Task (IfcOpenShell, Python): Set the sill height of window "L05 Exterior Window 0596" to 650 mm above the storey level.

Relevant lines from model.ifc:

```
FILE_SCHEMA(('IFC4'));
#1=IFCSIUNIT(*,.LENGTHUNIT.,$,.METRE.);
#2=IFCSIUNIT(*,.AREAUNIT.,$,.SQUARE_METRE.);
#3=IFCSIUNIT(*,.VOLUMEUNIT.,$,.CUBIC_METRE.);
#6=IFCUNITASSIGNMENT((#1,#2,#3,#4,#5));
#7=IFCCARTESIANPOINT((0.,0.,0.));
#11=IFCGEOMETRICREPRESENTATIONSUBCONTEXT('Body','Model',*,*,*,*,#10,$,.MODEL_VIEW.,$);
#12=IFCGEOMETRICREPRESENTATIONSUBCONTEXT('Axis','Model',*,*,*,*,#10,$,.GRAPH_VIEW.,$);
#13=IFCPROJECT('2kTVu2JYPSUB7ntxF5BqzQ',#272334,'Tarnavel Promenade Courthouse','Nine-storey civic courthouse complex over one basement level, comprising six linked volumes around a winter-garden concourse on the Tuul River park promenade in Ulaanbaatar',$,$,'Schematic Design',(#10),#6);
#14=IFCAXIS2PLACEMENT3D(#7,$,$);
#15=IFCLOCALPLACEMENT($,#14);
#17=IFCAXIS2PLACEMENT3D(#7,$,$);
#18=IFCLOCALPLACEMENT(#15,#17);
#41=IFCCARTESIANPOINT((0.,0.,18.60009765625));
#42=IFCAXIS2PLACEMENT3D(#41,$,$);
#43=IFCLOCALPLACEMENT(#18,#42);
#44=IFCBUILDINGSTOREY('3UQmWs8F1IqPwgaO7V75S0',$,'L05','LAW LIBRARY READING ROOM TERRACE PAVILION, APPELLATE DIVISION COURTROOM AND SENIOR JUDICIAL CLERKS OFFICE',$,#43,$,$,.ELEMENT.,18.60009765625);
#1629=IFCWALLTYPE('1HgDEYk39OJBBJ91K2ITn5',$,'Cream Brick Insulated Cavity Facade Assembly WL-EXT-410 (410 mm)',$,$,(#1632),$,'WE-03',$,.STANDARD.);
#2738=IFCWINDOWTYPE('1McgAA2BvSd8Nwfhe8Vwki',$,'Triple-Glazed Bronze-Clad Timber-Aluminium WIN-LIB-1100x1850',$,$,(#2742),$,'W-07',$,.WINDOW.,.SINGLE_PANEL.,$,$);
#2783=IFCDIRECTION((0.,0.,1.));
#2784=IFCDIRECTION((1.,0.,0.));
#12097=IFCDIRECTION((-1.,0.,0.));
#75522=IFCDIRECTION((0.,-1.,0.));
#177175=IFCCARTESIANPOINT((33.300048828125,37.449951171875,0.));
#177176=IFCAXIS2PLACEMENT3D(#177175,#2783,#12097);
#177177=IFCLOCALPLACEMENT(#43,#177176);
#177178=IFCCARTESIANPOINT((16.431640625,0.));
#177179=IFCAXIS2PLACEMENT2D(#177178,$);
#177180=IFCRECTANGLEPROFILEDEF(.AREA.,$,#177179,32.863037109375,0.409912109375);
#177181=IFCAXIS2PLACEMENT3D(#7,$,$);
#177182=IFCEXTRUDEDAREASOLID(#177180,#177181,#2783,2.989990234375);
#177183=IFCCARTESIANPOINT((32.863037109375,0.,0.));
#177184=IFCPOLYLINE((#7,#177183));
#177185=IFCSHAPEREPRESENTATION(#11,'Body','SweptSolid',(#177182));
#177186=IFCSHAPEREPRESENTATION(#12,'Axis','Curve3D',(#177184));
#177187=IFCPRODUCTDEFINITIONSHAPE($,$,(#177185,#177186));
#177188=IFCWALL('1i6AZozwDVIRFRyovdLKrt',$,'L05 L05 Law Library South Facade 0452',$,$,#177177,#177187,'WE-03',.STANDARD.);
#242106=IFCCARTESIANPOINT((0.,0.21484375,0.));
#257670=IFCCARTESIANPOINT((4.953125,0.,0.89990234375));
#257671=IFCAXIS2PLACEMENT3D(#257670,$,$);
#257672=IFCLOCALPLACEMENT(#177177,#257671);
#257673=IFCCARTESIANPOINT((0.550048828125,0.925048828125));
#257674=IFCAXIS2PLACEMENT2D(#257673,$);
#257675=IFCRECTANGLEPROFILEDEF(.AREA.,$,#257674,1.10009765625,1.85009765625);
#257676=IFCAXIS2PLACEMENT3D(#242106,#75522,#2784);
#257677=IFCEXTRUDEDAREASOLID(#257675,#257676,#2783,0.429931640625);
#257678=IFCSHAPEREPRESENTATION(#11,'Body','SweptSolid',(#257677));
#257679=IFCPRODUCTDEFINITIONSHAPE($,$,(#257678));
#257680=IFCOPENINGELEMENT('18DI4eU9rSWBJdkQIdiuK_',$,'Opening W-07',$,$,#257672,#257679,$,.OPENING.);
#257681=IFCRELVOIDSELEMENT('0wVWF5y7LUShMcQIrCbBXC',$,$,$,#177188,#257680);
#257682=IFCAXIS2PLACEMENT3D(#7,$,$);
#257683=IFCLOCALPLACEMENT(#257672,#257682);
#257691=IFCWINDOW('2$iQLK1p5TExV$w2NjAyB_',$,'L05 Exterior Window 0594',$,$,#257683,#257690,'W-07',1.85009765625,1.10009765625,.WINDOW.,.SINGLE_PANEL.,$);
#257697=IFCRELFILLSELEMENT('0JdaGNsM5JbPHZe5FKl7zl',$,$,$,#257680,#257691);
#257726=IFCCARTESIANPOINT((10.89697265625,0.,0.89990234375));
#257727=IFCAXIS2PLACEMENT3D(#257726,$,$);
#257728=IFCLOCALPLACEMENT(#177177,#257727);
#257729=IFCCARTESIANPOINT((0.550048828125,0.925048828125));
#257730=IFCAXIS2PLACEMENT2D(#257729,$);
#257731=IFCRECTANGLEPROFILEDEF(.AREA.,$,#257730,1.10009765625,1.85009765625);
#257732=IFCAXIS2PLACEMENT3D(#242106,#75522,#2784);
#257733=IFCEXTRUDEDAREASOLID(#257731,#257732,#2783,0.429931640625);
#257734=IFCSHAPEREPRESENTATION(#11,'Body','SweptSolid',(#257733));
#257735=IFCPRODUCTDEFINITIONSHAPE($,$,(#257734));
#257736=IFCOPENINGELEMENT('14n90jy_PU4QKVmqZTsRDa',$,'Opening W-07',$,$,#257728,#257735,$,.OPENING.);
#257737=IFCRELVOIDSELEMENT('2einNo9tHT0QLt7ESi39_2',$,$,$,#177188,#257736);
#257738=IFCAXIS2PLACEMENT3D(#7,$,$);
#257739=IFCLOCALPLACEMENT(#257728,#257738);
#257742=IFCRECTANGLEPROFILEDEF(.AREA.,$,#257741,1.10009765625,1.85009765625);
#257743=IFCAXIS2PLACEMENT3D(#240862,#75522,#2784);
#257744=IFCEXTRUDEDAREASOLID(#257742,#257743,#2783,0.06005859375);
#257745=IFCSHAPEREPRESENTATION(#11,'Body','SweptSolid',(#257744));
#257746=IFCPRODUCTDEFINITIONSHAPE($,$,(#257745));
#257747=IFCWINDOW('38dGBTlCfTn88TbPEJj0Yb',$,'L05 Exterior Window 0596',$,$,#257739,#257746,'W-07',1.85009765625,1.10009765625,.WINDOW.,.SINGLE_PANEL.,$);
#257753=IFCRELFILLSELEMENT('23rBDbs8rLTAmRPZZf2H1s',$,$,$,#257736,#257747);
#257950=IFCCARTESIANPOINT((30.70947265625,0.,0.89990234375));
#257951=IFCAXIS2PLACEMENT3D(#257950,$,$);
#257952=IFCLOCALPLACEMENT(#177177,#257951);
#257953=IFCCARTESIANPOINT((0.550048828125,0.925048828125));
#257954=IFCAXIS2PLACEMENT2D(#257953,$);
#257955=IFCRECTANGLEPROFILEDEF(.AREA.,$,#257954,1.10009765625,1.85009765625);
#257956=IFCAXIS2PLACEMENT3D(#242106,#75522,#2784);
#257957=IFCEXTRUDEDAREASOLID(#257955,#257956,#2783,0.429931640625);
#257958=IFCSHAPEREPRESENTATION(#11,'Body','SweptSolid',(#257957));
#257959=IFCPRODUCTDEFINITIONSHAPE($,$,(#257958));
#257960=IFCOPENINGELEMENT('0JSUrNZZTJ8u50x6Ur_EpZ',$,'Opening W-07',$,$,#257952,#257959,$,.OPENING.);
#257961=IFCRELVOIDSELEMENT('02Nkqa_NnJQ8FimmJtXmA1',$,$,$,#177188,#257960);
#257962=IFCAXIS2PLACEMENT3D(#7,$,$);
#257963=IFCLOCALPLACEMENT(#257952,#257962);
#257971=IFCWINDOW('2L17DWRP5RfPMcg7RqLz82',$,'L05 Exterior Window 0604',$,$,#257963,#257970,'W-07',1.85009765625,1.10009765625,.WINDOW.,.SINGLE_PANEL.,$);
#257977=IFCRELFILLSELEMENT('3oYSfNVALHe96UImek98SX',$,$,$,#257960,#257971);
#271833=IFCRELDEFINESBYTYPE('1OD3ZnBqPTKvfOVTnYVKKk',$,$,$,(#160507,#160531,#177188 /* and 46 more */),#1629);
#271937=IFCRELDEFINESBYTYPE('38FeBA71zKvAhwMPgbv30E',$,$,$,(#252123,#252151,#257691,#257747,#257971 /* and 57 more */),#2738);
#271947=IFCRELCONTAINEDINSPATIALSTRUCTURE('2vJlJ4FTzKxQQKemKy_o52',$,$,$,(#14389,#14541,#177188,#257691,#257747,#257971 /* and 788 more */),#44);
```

```python
import numpy as np
import ifcopenshell
import ifcopenshell.api.geometry
import ifcopenshell.geom
import ifcopenshell.util.element
import ifcopenshell.util.placement
import ifcopenshell.util.shape
import ifcopenshell.util.unit

model = ifcopenshell.open("model.ifc")
unit_scale = ifcopenshell.util.unit.calculate_unit_scale(model)

window = model.by_guid("38dGBTlCfTn88TbPEJj0Yb")
opening = window.FillsVoids[0].RelatingOpeningElement
storey = ifcopenshell.util.element.get_container(window, ifc_class="IfcBuildingStorey")
level = ifcopenshell.util.placement.get_local_placement(storey.ObjectPlacement)[2, 3]

# The opening's origin need not be at the sill, so measure its lowest point.
shape = ifcopenshell.geom.create_shape(ifcopenshell.geom.settings(), opening)
bottom = ifcopenshell.util.shape.get_shape_bottom_elevation(shape, shape.geometry) / unit_scale
dz = level + 0.65 / unit_scale - bottom

shift = np.array([0.0, 0.0, dz])
# The window is placed relative to its opening, so it follows when the opening moves.
matrix = ifcopenshell.util.placement.get_local_placement(opening.ObjectPlacement)
matrix[:3, 3] += shift
ifcopenshell.api.geometry.edit_object_placement(
    model, product=opening, matrix=matrix, is_si=False, should_transform_children=True
)

print(f"moved by {dz * unit_scale:+.3f} m")

model.write("model_edited.ifc")
```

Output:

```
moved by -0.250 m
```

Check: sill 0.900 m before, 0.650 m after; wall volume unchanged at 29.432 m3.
